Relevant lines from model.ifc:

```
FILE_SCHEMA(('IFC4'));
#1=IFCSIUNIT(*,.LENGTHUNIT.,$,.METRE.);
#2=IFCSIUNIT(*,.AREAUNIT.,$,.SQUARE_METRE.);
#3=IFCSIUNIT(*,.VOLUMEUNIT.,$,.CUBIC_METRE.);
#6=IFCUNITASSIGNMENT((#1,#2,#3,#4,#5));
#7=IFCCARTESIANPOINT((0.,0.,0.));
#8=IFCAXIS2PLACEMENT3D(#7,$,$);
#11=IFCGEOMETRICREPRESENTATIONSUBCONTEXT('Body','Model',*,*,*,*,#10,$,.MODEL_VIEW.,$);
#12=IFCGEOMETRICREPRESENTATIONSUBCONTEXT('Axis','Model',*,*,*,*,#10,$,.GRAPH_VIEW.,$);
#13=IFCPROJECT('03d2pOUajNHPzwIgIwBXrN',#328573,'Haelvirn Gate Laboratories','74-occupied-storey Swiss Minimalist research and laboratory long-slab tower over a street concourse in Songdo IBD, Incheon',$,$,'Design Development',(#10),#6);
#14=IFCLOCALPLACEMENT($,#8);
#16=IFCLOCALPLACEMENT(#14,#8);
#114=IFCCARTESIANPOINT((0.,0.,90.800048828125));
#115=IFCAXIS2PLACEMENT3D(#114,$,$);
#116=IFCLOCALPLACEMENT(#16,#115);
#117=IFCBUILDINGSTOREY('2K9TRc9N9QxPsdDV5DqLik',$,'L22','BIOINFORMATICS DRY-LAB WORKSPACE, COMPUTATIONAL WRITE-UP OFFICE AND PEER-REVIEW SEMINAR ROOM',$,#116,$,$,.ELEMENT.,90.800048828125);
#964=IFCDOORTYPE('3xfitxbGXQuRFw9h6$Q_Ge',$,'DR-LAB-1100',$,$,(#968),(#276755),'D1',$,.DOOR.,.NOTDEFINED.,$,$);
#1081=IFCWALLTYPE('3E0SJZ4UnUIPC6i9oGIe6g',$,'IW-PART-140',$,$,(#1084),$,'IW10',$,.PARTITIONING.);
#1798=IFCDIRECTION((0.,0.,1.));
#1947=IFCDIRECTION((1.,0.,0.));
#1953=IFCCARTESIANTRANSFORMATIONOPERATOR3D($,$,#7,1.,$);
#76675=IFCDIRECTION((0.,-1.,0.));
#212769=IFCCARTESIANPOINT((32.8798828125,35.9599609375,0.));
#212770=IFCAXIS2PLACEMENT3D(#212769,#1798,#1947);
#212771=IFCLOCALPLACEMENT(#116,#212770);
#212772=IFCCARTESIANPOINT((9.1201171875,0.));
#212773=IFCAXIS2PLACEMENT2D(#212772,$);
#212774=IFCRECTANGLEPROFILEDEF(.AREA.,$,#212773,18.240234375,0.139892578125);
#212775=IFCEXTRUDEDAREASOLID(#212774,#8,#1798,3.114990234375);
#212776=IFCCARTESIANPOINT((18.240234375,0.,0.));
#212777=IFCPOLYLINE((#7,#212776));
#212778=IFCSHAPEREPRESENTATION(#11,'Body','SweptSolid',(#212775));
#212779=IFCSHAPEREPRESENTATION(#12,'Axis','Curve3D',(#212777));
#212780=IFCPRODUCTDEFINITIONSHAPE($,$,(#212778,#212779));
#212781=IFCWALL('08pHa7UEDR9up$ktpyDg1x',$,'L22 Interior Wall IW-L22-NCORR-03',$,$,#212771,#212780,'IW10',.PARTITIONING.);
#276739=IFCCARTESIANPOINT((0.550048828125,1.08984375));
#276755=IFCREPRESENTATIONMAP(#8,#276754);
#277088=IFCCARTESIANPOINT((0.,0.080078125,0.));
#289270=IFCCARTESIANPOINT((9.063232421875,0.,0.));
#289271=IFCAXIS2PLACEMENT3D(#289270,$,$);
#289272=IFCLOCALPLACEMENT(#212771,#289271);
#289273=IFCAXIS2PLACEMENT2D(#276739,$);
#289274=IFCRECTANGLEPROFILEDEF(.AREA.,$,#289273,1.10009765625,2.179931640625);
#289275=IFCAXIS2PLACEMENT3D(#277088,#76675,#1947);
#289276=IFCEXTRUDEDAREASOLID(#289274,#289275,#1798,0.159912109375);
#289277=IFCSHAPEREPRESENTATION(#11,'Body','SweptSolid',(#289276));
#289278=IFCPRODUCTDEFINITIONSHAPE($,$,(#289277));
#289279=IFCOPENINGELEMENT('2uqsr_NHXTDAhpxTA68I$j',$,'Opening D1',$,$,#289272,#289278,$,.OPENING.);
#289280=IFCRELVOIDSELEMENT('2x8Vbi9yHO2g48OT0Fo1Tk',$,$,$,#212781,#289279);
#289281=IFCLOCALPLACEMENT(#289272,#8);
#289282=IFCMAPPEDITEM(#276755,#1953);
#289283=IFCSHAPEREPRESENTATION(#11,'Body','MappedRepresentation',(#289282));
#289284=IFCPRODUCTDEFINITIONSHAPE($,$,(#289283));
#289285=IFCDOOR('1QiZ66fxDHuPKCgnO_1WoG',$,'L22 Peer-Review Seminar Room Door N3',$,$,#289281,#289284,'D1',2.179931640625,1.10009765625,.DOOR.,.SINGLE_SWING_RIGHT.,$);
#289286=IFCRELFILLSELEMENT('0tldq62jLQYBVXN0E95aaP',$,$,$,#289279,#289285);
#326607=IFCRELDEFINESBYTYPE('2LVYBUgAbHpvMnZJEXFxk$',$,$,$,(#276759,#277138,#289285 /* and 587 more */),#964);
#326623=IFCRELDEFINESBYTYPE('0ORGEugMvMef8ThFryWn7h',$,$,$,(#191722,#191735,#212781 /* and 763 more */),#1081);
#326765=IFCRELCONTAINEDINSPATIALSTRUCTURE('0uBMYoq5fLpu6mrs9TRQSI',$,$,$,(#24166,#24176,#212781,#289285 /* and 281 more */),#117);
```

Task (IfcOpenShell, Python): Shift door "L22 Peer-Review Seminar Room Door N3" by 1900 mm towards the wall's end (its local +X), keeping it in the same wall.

```python
import ifcopenshell
import ifcopenshell.api.geometry
import ifcopenshell.util.placement

model = ifcopenshell.open("model.ifc")

door = model.by_guid("1QiZ66fxDHuPKCgnO_1WoG")
opening = door.FillsVoids[0].RelatingOpeningElement
wall = opening.VoidsElements[0].RelatingBuildingElement

wall_matrix = ifcopenshell.util.placement.get_local_placement(wall.ObjectPlacement)
shift = wall_matrix[:3, 0] * 1.9
before = ifcopenshell.util.placement.get_local_placement(door.ObjectPlacement)[:3, 3].copy()

# The door is placed relative to its opening, so it follows when the opening moves.
matrix = ifcopenshell.util.placement.get_local_placement(opening.ObjectPlacement)
matrix[:3, 3] += shift
ifcopenshell.api.geometry.edit_object_placement(
    model, product=opening, matrix=matrix, is_si=False, should_transform_children=True
)

after = ifcopenshell.util.placement.get_local_placement(door.ObjectPlacement)[:3, 3]
print("door moved by", (after - before).round(3) + 0.0)

model.write("model_rev.ifc")
```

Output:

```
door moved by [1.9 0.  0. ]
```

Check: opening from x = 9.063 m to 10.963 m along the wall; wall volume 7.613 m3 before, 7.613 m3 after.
